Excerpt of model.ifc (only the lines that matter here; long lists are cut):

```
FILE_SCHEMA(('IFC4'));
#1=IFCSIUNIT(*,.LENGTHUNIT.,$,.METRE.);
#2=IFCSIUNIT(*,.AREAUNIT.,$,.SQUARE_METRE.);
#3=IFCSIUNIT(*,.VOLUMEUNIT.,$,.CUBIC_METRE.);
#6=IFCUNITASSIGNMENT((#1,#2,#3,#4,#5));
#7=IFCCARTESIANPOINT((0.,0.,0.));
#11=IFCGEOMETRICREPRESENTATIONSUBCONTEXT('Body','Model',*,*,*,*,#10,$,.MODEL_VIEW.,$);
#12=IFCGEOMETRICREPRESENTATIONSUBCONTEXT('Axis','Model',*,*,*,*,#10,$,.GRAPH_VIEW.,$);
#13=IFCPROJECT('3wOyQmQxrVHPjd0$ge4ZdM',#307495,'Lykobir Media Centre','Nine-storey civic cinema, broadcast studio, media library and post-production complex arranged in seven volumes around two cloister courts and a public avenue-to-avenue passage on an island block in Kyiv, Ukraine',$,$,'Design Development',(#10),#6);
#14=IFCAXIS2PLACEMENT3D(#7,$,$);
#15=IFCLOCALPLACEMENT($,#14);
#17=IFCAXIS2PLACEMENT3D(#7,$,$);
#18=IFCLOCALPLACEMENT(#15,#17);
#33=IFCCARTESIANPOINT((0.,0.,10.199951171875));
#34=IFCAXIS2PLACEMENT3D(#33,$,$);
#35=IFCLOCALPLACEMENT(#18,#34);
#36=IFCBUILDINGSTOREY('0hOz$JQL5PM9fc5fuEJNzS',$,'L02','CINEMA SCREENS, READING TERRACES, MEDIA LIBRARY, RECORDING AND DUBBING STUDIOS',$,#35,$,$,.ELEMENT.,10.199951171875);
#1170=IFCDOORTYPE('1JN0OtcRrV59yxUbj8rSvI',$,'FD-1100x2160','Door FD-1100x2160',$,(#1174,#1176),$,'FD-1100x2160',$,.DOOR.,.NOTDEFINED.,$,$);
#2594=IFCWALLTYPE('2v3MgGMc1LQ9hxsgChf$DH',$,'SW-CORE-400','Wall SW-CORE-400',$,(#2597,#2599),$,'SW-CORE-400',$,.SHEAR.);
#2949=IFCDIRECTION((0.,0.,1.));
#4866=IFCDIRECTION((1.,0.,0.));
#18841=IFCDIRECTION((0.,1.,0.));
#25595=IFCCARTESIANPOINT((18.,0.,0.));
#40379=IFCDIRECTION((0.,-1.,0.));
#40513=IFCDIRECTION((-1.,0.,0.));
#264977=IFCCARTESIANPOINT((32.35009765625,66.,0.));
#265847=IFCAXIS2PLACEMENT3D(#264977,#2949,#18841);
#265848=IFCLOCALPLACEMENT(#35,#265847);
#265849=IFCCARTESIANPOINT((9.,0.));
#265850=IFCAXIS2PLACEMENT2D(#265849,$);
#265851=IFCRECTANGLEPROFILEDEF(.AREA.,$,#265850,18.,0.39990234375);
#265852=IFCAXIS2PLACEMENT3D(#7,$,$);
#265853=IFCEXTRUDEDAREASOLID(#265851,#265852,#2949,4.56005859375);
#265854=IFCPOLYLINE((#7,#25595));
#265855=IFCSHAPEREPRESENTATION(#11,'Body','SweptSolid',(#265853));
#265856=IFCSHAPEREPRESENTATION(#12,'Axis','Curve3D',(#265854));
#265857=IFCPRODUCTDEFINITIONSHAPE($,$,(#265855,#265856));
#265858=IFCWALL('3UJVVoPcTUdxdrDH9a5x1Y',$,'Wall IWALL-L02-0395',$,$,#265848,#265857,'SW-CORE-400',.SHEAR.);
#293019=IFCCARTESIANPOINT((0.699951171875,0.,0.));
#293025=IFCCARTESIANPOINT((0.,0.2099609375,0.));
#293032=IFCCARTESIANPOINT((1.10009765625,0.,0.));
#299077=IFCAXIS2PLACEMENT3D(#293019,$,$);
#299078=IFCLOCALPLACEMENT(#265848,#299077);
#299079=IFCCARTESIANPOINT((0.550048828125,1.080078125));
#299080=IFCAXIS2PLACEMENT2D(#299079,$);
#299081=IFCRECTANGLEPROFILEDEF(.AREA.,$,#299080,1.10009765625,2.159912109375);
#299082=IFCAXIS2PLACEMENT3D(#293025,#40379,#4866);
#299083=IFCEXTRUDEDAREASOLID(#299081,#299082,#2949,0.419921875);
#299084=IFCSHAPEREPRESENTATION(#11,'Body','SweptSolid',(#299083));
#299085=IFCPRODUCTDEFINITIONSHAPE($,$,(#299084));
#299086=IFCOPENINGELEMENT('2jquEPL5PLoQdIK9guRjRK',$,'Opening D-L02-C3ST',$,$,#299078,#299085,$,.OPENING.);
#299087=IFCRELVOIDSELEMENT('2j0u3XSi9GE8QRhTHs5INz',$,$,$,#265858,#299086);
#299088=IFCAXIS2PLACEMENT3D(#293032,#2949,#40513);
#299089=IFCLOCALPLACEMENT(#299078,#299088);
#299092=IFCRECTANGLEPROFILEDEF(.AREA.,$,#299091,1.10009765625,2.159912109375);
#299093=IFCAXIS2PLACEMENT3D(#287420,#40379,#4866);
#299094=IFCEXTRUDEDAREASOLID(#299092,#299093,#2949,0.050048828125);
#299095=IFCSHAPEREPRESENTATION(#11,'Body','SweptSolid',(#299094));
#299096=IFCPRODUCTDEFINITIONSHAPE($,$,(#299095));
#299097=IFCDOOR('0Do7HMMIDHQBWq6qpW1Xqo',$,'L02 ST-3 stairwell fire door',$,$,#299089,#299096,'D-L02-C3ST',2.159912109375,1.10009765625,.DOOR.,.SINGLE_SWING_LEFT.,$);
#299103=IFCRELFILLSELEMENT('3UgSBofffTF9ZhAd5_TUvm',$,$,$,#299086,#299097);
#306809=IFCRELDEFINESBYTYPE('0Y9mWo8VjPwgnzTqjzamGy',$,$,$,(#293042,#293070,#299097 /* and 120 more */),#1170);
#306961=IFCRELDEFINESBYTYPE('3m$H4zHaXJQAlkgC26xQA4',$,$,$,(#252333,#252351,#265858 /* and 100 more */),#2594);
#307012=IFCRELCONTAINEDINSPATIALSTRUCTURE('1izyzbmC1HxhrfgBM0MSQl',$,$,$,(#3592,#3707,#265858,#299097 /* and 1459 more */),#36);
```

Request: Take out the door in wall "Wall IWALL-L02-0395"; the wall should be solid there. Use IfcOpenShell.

```python
import ifcopenshell
import ifcopenshell.api.feature
import ifcopenshell.api.root
import ifcopenshell.geom
import ifcopenshell.util.shape

model = ifcopenshell.open("model.ifc")
settings = ifcopenshell.geom.settings()


def volume(element):
    """Net volume in cubic metres, openings subtracted."""
    shape = ifcopenshell.geom.create_shape(settings, element)
    return ifcopenshell.util.shape.get_volume(shape.geometry)


door = model.by_guid("0Do7HMMIDHQBWq6qpW1Xqo")
opening = door.FillsVoids[0].RelatingOpeningElement
wall = opening.VoidsElements[0].RelatingBuildingElement
before = volume(wall)

ifcopenshell.api.root.remove_product(model, product=door)
ifcopenshell.api.feature.remove_feature(model, feature=opening)

after = volume(wall)

print(f"wall volume {before:.3f} -> {after:.3f} m3")

model.write("model_rev.ifc")
```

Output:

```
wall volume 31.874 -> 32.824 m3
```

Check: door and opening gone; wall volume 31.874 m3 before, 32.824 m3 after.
